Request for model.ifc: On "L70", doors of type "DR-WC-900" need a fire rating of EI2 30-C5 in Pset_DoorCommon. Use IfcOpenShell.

First a look at what the model holds.

```python
import ifcopenshell
import ifcopenshell.util.element

model = ifcopenshell.open("model.ifc")
print(model.schema)
storey = next(s for s in model.by_type("IfcBuildingStorey") if s.Name == "L70")
doors = [e for e in ifcopenshell.util.element.get_decomposition(storey) if e.is_a("IfcDoor")]
seen = {}
for e in doors:
    element_type = ifcopenshell.util.element.get_type(e)
    key = (element_type.Name if element_type != e and element_type else None, ifcopenshell.util.element.get_pset(e, "Pset_DoorCommon", "FireRating"))
    seen[key] = seen.get(key, 0) + 1
for (name, value), count in sorted(seen.items(), key=str):
    print(count, "x", name, "|", value)
```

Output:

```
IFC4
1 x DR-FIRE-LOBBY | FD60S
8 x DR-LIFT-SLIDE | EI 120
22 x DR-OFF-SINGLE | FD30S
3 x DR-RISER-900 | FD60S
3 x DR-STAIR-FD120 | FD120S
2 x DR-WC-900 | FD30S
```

```python
import ifcopenshell
import ifcopenshell.api.pset
import ifcopenshell.util.element

model = ifcopenshell.open("model.ifc")

storey = next(s for s in model.by_type("IfcBuildingStorey") if s.Name == "L70")
doors = [e for e in ifcopenshell.util.element.get_decomposition(storey) if e.is_a("IfcDoor")]

count = 0
for e in doors:
    element_type = ifcopenshell.util.element.get_type(e)
    if element_type in (None, e) or element_type.Name != "DR-WC-900":
        continue
    found = ifcopenshell.util.element.get_pset(e, "Pset_DoorCommon", should_inherit=False)
    if found:
        pset = model.by_id(found["id"])
        if len(ifcopenshell.util.element.get_elements_by_pset(pset)) > 1:
            pset = ifcopenshell.api.pset.unshare_pset(model, products=[e], pset=pset)[0]
    else:
        pset = ifcopenshell.api.pset.add_pset(model, product=e, name="Pset_DoorCommon")
    ifcopenshell.api.pset.edit_pset(model, pset=pset, properties={"FireRating": "EI2 30-C5"})
    count += 1

print(count, "doors updated")

model.write("model-out.ifc")
```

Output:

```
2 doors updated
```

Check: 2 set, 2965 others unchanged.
